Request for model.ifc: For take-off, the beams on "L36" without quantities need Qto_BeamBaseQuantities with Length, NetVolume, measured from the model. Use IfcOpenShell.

First a look at what the model holds.

```python
import ifcopenshell
import ifcopenshell.util.element
import ifcopenshell.util.unit

model = ifcopenshell.open("model.ifc")
print(model.schema)
for unit_type in ("LENGTHUNIT", "AREAUNIT", "VOLUMEUNIT"):
    print(unit_type, ifcopenshell.util.unit.calculate_unit_scale(model, unit_type))
storey = next(s for s in model.by_type("IfcBuildingStorey") if s.Name == "L36")
beams = [e for e in ifcopenshell.util.element.get_decomposition(storey) if e.is_a("IfcBeam")]
for e in sorted(beams, key=lambda e: e.id()):
    print(e.id(), e.is_a(), e.Name, list(ifcopenshell.util.element.get_psets(e, qtos_only=True)), sep=" | ")
```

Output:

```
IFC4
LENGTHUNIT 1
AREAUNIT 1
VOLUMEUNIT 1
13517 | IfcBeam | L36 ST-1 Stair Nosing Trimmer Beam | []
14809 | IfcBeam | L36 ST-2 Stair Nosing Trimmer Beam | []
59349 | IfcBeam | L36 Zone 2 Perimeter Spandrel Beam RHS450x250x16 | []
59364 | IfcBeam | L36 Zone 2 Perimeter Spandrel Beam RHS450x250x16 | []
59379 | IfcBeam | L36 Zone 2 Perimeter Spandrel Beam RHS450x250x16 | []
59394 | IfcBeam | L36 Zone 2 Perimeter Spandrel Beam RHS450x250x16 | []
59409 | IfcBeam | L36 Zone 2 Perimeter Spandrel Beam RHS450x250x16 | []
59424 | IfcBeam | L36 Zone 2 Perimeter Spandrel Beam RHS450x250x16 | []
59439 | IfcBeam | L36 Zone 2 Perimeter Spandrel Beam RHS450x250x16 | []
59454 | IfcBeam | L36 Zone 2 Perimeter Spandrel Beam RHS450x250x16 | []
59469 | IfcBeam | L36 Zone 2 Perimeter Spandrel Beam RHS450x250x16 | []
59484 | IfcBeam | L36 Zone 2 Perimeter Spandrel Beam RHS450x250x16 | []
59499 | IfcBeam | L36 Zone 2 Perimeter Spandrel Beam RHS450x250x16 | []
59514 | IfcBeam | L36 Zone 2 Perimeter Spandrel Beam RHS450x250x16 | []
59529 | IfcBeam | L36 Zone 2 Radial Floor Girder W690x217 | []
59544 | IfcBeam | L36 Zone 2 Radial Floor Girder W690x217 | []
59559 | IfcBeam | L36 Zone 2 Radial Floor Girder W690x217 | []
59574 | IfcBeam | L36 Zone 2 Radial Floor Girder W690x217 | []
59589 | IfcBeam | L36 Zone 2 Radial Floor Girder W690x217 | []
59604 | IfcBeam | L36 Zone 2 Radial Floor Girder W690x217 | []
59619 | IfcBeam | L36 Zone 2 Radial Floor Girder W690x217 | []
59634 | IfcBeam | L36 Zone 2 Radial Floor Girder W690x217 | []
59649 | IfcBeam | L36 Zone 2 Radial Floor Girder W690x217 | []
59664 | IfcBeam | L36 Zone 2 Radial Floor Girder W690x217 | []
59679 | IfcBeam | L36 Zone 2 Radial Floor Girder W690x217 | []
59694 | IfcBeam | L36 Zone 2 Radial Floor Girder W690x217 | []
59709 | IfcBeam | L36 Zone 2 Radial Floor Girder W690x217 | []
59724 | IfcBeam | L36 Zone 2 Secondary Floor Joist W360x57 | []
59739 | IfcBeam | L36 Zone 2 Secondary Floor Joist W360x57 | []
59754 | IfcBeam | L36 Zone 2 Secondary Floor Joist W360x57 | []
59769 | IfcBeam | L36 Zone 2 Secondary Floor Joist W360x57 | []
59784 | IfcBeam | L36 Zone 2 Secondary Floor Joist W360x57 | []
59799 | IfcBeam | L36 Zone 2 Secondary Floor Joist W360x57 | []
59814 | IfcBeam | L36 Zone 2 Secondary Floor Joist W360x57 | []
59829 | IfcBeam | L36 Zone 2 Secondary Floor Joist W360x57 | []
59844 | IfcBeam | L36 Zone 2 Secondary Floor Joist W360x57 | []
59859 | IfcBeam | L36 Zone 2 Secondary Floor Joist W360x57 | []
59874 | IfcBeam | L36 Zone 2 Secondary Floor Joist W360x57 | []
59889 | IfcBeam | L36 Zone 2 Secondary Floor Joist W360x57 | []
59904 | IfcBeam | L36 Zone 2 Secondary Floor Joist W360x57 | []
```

```python
import ifcopenshell
import ifcopenshell.api.pset
import ifcopenshell.geom
import ifcopenshell.util.element
import ifcopenshell.util.shape
import ifcopenshell.util.unit

model = ifcopenshell.open("model.ifc")
unit_scale = ifcopenshell.util.unit.calculate_unit_scale(model)
volume_scale = ifcopenshell.util.unit.calculate_unit_scale(model, "VOLUMEUNIT")
settings = ifcopenshell.geom.settings()

storey = next(s for s in model.by_type("IfcBuildingStorey") if s.Name == "L36")
beams = [e for e in ifcopenshell.util.element.get_decomposition(storey) if e.is_a("IfcBeam")]

for e in sorted(beams, key=lambda e: e.id()):
    if ifcopenshell.util.element.get_psets(e, qtos_only=True, should_inherit=False):
        continue
    # Geometry comes back in metres, in the element's own axes.
    shape = ifcopenshell.geom.create_shape(settings, e)
    values = {
        "Length": ifcopenshell.util.shape.get_max_xyz(shape.geometry) / unit_scale,
        "NetVolume": ifcopenshell.util.shape.get_volume(shape.geometry) / volume_scale,
    }
    qto = ifcopenshell.api.pset.add_qto(model, product=e, name="Qto_BeamBaseQuantities")
    ifcopenshell.api.pset.edit_qto(model, qto=qto, properties=values)
    print(e.id(), {k: round(v, 3) for k, v in values.items()})

model.write("model-out.ifc")
```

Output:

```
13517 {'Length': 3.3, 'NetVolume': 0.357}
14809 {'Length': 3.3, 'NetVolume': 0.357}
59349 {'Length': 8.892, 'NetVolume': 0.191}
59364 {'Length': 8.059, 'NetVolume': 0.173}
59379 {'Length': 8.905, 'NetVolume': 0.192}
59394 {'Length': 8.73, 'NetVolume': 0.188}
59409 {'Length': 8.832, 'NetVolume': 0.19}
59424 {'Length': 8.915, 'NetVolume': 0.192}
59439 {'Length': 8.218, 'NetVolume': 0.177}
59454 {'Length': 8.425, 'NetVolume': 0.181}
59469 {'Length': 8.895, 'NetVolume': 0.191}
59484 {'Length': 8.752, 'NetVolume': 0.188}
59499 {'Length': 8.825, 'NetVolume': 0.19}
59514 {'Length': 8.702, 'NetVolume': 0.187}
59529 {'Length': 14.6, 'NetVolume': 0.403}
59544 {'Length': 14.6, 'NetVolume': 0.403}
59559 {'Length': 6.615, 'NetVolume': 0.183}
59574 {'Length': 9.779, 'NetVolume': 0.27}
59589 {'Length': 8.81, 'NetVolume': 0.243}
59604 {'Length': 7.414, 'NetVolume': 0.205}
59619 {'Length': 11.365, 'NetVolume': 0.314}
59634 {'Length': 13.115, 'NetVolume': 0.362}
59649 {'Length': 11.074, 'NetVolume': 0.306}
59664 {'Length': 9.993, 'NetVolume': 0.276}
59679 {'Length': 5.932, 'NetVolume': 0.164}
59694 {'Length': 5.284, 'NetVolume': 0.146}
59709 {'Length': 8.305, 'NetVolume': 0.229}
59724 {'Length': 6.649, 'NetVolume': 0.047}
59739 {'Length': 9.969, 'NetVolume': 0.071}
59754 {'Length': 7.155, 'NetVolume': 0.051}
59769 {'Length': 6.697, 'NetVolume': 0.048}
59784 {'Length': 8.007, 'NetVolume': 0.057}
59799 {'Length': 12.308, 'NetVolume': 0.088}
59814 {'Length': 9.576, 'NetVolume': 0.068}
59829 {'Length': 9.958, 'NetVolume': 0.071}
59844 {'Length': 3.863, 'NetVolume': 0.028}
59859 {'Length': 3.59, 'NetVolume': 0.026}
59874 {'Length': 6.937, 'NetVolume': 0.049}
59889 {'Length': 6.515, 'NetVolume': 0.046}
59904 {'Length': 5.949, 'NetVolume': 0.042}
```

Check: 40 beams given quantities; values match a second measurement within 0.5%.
